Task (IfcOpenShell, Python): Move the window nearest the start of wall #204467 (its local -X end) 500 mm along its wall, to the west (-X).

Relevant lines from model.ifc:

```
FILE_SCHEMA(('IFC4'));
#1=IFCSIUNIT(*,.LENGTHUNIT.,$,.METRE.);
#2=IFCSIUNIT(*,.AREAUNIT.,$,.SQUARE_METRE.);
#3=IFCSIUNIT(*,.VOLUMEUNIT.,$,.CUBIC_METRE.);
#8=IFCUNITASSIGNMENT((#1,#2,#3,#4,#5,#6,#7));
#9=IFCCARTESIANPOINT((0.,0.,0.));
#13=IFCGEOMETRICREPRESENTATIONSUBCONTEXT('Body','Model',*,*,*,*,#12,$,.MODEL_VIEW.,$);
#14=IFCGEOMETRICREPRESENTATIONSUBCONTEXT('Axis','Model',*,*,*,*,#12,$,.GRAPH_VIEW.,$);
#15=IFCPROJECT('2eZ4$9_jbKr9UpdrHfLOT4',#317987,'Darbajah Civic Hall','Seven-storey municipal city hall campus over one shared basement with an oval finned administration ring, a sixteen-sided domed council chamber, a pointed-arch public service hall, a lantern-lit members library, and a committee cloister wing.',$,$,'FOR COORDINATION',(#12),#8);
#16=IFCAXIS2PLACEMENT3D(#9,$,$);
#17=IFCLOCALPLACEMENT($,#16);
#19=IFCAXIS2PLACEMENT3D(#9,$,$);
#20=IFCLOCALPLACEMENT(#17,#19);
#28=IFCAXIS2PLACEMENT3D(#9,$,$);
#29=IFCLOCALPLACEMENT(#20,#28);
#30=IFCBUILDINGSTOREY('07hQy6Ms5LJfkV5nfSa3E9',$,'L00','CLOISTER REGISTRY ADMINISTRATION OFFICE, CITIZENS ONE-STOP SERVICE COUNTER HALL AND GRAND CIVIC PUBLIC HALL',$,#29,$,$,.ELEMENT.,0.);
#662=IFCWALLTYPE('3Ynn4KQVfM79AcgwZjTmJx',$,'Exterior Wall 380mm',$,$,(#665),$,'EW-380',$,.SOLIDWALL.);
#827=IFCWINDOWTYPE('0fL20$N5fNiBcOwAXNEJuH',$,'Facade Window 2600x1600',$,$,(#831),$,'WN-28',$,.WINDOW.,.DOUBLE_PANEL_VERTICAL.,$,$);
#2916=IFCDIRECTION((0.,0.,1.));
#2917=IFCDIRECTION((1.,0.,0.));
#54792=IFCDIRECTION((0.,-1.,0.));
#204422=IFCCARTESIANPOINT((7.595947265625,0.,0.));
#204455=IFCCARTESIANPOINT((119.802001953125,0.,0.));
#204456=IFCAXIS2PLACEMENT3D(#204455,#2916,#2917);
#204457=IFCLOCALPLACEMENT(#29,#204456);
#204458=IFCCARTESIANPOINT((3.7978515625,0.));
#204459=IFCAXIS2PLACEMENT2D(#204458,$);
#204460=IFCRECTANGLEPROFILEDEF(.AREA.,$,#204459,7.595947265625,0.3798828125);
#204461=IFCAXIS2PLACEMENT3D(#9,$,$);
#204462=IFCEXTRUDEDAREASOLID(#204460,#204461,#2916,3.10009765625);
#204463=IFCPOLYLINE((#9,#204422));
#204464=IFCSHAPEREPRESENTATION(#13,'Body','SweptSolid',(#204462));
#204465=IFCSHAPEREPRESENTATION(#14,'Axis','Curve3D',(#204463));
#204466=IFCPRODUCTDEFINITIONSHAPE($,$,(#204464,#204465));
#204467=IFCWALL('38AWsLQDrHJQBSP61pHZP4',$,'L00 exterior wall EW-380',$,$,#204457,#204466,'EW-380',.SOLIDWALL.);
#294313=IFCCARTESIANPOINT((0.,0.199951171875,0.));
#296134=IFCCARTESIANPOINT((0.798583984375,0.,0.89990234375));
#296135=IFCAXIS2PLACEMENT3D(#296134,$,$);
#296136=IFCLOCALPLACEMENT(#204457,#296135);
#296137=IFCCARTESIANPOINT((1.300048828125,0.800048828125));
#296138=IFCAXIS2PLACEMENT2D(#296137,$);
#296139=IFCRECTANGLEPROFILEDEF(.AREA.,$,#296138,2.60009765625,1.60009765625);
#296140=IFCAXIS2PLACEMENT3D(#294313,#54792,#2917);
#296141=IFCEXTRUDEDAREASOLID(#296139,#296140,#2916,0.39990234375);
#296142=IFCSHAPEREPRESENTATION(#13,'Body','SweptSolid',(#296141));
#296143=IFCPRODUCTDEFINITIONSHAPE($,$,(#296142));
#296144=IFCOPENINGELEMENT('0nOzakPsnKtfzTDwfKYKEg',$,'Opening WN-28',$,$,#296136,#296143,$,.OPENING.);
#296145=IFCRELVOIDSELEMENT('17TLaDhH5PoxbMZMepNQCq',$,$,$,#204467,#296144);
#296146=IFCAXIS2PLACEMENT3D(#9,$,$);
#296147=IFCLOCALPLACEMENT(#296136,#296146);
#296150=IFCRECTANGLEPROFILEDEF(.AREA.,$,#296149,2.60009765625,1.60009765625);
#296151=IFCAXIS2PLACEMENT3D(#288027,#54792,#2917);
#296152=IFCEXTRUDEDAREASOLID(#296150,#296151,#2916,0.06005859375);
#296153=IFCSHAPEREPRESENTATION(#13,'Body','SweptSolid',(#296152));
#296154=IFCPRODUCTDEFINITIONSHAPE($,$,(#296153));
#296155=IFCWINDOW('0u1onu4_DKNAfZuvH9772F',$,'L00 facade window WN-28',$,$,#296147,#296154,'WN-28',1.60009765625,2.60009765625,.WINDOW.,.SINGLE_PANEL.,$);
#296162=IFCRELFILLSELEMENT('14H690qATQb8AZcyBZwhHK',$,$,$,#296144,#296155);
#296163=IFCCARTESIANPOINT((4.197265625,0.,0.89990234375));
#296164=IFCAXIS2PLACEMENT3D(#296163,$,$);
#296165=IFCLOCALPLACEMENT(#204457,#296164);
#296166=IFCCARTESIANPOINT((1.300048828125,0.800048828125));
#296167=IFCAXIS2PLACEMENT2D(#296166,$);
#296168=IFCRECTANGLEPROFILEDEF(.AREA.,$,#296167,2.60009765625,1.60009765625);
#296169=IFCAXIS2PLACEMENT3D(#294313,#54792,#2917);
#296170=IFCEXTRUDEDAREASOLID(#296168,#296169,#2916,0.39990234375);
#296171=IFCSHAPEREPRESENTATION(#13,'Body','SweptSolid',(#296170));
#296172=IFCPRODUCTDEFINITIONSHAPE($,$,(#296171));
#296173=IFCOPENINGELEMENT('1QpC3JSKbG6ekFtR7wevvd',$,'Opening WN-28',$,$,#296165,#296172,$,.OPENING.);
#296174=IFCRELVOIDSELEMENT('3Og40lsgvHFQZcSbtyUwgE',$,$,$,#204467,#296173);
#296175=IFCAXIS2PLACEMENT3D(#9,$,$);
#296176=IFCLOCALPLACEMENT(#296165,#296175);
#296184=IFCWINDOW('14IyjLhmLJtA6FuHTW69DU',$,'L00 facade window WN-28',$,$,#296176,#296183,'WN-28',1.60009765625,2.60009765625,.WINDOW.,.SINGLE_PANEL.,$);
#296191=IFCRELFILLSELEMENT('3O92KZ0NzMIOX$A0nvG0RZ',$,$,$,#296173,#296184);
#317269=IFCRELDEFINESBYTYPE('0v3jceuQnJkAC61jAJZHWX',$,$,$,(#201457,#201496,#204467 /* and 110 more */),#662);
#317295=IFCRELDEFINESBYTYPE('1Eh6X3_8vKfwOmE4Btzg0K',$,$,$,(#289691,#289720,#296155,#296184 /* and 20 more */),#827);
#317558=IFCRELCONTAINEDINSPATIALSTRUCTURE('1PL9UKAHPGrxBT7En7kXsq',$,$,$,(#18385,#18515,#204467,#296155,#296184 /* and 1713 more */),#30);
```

```python
import ifcopenshell
import ifcopenshell.api.geometry
import ifcopenshell.util.placement
import ifcopenshell.util.unit

model = ifcopenshell.open("model.ifc")
unit_scale = ifcopenshell.util.unit.calculate_unit_scale(model)

window = model.by_guid("0u1onu4_DKNAfZuvH9772F")
opening = window.FillsVoids[0].RelatingOpeningElement
wall = opening.VoidsElements[0].RelatingBuildingElement

wall_matrix = ifcopenshell.util.placement.get_local_placement(wall.ObjectPlacement)
shift = wall_matrix[:3, 0] * -0.5 / unit_scale
before = ifcopenshell.util.placement.get_local_placement(window.ObjectPlacement)[:3, 3].copy()

# The window is placed relative to its opening, so it follows when the opening moves.
matrix = ifcopenshell.util.placement.get_local_placement(opening.ObjectPlacement)
matrix[:3, 3] += shift
ifcopenshell.api.geometry.edit_object_placement(
    model, product=opening, matrix=matrix, is_si=False, should_transform_children=True
)

after = ifcopenshell.util.placement.get_local_placement(window.ObjectPlacement)[:3, 3]
print("window moved by", (after - before).round(3) + 0.0)

model.write("model_v2.ifc")
```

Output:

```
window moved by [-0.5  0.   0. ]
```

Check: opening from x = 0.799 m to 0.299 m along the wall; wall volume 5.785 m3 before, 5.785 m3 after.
